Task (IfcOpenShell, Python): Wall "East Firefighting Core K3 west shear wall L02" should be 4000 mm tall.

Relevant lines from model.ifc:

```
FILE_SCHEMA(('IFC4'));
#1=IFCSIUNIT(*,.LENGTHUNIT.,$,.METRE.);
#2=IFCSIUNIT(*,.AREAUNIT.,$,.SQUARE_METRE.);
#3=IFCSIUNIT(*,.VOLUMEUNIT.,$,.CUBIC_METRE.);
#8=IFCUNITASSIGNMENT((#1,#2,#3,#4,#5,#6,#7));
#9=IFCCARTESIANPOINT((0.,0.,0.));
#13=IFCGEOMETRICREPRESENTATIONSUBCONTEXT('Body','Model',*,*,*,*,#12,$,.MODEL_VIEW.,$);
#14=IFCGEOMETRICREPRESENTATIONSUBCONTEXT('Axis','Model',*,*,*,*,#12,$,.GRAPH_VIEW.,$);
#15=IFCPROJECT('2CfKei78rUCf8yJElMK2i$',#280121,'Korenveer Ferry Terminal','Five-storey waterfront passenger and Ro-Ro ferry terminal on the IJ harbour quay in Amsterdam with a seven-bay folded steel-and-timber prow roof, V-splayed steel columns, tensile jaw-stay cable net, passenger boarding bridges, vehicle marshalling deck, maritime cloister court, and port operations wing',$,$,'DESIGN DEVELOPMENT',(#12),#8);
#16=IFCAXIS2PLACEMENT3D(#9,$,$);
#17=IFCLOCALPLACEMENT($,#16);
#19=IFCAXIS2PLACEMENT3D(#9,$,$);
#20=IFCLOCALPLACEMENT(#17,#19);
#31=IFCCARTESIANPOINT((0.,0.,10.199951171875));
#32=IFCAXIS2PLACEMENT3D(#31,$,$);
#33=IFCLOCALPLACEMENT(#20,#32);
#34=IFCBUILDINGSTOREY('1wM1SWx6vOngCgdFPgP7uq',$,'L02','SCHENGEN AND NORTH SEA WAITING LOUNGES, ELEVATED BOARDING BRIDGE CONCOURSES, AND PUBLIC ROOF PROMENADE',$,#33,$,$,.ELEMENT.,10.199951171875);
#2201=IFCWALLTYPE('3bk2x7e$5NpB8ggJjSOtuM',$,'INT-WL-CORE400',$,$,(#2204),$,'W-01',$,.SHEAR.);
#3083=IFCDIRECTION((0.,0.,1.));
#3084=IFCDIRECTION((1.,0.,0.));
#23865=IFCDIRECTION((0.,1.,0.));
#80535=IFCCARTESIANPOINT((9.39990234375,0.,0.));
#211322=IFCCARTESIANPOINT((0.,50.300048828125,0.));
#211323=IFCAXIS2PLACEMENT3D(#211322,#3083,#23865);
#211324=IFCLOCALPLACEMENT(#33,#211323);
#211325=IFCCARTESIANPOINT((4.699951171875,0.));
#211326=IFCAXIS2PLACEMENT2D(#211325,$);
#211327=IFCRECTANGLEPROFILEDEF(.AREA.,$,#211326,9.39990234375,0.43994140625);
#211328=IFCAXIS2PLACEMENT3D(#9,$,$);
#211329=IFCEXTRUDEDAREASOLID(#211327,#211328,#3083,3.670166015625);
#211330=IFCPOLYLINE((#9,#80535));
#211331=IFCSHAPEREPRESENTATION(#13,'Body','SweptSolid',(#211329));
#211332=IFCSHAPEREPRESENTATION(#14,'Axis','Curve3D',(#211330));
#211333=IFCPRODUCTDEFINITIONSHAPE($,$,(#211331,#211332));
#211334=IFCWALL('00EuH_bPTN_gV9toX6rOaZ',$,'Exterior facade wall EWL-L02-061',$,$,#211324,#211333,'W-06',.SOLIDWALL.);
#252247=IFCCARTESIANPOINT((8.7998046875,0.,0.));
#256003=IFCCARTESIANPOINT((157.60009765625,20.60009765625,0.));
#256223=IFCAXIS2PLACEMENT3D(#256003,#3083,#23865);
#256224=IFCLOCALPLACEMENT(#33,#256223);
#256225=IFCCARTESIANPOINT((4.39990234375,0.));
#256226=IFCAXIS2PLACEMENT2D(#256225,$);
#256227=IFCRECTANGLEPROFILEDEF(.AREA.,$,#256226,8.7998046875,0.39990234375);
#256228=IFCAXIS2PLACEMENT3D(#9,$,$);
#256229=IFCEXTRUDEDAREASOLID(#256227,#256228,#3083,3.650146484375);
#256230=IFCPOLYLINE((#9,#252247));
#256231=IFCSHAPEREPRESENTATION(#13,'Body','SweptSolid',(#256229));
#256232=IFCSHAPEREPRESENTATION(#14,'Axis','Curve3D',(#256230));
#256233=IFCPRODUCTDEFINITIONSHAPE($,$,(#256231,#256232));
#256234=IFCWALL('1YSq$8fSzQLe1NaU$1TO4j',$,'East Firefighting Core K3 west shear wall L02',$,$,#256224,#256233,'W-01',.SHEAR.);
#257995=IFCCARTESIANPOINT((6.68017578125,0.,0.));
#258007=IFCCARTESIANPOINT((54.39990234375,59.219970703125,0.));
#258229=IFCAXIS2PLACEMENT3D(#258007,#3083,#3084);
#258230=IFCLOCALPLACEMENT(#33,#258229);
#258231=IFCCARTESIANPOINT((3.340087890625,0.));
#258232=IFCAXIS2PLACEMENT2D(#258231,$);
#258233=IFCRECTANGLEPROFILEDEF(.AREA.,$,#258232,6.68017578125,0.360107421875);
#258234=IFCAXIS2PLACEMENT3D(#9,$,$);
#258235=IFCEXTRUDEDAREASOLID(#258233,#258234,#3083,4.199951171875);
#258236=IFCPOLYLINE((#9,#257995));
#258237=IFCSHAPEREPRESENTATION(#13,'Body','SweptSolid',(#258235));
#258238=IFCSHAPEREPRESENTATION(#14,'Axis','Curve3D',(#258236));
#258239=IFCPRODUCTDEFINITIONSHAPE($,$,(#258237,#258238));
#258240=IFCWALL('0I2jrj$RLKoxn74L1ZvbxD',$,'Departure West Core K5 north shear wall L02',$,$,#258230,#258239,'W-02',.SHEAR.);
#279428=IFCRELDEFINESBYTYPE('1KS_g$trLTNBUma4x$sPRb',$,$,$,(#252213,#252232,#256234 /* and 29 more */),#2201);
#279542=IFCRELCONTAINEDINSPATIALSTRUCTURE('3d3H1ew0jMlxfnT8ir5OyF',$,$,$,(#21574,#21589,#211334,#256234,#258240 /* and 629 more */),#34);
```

```python
import ifcopenshell
import ifcopenshell.geom
import ifcopenshell.util.representation
import ifcopenshell.util.shape

model = ifcopenshell.open("model.ifc")
settings = ifcopenshell.geom.settings()


def volume(element):
    """Net volume in cubic metres, openings subtracted."""
    shape = ifcopenshell.geom.create_shape(settings, element)
    return ifcopenshell.util.shape.get_volume(shape.geometry)


wall = model.by_id(256234)
before = volume(wall)

body = ifcopenshell.util.representation.get_representation(wall, "Model", "Body")
solid = body.Items[0]
old_height = solid.Depth
solid.Depth = 4.0
after = volume(wall)

print(f"height {old_height:g} -> {solid.Depth:g}, volume {before:.3f} -> {after:.3f} m3")

model.write("model_v2.ifc")
```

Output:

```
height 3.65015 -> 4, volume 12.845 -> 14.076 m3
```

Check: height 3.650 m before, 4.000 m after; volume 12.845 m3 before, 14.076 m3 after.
